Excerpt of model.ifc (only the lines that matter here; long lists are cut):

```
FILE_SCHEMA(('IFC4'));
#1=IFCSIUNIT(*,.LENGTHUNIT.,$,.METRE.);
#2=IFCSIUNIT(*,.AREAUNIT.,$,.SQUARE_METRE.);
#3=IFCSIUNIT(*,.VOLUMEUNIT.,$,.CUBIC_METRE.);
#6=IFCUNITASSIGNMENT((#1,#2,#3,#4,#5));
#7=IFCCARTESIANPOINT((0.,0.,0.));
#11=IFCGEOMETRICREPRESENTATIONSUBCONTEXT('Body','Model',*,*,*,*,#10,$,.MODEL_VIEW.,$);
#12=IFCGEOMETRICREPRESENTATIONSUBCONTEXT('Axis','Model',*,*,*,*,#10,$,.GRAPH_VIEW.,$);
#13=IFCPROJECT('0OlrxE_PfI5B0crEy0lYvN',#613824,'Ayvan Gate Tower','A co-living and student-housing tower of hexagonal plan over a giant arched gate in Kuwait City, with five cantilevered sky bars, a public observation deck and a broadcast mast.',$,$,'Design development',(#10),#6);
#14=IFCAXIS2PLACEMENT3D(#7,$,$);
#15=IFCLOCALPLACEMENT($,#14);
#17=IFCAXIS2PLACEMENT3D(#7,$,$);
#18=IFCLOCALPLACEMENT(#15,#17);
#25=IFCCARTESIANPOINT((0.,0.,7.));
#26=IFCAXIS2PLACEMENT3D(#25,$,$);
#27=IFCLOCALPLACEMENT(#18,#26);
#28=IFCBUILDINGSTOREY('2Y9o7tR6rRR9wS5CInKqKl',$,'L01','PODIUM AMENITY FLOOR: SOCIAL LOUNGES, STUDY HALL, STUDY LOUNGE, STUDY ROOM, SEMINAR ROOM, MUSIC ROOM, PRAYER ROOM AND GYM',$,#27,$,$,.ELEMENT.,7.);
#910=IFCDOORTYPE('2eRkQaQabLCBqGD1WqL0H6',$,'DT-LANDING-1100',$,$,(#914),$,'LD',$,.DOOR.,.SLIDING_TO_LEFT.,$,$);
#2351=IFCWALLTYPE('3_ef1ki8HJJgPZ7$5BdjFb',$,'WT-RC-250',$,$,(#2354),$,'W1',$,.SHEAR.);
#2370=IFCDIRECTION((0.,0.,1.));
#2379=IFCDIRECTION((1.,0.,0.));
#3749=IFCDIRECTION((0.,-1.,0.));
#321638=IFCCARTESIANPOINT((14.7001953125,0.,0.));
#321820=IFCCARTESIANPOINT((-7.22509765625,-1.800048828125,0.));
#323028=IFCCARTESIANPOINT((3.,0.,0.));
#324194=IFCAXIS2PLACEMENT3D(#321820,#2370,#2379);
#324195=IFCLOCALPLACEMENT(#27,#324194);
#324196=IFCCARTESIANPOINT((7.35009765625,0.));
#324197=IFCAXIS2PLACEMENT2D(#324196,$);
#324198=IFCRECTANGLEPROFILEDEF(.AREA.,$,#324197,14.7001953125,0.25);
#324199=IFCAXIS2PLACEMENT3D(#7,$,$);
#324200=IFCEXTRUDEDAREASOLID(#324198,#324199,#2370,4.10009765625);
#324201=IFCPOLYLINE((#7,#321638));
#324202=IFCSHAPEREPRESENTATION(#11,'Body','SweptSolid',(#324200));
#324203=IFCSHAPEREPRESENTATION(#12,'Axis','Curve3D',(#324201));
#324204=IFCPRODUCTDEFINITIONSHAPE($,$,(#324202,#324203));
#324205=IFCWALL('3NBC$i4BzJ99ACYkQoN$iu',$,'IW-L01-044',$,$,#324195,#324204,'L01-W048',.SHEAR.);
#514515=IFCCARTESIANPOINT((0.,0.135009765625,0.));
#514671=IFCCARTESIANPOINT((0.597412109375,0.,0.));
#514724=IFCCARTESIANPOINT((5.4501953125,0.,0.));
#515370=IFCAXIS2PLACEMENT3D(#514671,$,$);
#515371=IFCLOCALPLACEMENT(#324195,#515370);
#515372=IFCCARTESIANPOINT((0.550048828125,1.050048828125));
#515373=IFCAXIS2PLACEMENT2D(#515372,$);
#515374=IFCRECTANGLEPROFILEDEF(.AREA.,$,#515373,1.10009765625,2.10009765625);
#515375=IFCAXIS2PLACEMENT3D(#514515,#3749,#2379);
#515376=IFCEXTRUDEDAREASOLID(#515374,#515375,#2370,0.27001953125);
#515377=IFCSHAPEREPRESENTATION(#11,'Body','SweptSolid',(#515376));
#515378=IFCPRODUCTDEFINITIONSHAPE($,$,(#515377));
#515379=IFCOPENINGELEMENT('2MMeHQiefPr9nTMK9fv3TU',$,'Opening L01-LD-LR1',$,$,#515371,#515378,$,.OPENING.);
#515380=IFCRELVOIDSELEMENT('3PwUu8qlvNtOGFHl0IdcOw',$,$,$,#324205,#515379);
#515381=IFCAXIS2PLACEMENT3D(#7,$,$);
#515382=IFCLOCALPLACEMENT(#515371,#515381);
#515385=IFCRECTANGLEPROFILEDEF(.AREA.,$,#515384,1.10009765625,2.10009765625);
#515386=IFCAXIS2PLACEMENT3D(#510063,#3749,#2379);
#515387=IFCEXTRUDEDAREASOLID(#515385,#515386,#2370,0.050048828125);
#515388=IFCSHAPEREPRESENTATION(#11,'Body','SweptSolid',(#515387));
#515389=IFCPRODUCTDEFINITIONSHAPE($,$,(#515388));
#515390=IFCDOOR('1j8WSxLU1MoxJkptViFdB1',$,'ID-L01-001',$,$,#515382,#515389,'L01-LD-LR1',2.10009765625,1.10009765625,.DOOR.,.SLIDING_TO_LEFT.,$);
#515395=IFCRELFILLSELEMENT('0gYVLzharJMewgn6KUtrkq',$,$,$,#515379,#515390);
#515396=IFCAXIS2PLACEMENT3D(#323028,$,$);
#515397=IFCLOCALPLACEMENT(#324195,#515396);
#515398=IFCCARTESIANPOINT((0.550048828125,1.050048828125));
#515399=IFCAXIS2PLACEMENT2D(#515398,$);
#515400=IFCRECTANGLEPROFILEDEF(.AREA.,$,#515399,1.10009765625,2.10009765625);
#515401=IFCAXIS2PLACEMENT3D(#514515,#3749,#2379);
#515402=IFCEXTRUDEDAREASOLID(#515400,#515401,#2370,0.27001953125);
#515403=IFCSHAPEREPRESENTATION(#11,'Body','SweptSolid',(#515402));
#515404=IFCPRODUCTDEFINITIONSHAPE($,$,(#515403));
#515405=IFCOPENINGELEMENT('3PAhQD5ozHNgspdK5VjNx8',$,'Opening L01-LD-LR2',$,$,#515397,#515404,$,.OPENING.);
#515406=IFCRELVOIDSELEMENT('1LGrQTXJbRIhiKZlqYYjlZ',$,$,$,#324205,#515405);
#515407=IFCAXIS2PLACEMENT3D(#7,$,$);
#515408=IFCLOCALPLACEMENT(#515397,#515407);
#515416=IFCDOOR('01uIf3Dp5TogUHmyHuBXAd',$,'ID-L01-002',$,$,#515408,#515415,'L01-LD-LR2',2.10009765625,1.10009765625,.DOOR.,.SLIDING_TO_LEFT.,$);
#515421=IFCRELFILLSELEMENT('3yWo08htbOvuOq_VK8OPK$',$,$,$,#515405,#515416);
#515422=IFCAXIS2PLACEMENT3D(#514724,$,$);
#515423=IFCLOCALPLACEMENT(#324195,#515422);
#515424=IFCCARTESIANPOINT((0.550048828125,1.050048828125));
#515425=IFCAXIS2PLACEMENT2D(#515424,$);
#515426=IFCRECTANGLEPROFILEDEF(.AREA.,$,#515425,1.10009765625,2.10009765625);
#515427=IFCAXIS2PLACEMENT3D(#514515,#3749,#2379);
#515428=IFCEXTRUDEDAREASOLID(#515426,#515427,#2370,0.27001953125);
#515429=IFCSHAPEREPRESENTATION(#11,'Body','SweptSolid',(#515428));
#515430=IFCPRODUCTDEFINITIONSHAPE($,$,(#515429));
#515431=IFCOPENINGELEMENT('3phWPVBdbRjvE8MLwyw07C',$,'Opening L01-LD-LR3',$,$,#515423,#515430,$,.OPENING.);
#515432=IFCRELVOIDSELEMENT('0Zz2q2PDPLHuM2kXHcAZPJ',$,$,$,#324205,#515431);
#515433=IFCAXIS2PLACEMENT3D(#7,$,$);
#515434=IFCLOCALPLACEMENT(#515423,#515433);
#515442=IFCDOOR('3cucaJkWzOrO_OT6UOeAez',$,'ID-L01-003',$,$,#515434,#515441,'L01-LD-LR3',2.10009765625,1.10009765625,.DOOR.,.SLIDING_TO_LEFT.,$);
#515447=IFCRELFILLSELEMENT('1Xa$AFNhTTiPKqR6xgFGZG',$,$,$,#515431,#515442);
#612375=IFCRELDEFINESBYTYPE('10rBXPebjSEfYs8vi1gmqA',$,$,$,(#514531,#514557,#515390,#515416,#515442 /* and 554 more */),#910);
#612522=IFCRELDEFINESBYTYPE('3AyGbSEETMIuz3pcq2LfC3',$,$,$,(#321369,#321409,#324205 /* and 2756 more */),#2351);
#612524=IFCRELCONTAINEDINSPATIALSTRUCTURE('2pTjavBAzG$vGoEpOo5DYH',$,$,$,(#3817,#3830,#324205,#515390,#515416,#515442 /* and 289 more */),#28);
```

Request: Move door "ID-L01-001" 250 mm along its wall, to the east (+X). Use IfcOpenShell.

```python
import ifcopenshell
import ifcopenshell.api.geometry
import ifcopenshell.util.placement
import ifcopenshell.util.unit

model = ifcopenshell.open("model.ifc")
unit_scale = ifcopenshell.util.unit.calculate_unit_scale(model)

door = model.by_guid("1j8WSxLU1MoxJkptViFdB1")
opening = door.FillsVoids[0].RelatingOpeningElement
wall = opening.VoidsElements[0].RelatingBuildingElement

wall_matrix = ifcopenshell.util.placement.get_local_placement(wall.ObjectPlacement)
shift = wall_matrix[:3, 0] * 0.25 / unit_scale
before = ifcopenshell.util.placement.get_local_placement(door.ObjectPlacement)[:3, 3].copy()

# The door is placed relative to its opening, so it follows when the opening moves.
matrix = ifcopenshell.util.placement.get_local_placement(opening.ObjectPlacement)
matrix[:3, 3] += shift
ifcopenshell.api.geometry.edit_object_placement(
    model, product=opening, matrix=matrix, is_si=False, should_transform_children=True
)

after = ifcopenshell.util.placement.get_local_placement(door.ObjectPlacement)[:3, 3]
print("door moved by", (after - before).round(3) + 0.0)

model.write("model_rev.ifc")
```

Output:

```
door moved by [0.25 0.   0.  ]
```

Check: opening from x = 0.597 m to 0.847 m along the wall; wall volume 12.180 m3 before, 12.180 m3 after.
